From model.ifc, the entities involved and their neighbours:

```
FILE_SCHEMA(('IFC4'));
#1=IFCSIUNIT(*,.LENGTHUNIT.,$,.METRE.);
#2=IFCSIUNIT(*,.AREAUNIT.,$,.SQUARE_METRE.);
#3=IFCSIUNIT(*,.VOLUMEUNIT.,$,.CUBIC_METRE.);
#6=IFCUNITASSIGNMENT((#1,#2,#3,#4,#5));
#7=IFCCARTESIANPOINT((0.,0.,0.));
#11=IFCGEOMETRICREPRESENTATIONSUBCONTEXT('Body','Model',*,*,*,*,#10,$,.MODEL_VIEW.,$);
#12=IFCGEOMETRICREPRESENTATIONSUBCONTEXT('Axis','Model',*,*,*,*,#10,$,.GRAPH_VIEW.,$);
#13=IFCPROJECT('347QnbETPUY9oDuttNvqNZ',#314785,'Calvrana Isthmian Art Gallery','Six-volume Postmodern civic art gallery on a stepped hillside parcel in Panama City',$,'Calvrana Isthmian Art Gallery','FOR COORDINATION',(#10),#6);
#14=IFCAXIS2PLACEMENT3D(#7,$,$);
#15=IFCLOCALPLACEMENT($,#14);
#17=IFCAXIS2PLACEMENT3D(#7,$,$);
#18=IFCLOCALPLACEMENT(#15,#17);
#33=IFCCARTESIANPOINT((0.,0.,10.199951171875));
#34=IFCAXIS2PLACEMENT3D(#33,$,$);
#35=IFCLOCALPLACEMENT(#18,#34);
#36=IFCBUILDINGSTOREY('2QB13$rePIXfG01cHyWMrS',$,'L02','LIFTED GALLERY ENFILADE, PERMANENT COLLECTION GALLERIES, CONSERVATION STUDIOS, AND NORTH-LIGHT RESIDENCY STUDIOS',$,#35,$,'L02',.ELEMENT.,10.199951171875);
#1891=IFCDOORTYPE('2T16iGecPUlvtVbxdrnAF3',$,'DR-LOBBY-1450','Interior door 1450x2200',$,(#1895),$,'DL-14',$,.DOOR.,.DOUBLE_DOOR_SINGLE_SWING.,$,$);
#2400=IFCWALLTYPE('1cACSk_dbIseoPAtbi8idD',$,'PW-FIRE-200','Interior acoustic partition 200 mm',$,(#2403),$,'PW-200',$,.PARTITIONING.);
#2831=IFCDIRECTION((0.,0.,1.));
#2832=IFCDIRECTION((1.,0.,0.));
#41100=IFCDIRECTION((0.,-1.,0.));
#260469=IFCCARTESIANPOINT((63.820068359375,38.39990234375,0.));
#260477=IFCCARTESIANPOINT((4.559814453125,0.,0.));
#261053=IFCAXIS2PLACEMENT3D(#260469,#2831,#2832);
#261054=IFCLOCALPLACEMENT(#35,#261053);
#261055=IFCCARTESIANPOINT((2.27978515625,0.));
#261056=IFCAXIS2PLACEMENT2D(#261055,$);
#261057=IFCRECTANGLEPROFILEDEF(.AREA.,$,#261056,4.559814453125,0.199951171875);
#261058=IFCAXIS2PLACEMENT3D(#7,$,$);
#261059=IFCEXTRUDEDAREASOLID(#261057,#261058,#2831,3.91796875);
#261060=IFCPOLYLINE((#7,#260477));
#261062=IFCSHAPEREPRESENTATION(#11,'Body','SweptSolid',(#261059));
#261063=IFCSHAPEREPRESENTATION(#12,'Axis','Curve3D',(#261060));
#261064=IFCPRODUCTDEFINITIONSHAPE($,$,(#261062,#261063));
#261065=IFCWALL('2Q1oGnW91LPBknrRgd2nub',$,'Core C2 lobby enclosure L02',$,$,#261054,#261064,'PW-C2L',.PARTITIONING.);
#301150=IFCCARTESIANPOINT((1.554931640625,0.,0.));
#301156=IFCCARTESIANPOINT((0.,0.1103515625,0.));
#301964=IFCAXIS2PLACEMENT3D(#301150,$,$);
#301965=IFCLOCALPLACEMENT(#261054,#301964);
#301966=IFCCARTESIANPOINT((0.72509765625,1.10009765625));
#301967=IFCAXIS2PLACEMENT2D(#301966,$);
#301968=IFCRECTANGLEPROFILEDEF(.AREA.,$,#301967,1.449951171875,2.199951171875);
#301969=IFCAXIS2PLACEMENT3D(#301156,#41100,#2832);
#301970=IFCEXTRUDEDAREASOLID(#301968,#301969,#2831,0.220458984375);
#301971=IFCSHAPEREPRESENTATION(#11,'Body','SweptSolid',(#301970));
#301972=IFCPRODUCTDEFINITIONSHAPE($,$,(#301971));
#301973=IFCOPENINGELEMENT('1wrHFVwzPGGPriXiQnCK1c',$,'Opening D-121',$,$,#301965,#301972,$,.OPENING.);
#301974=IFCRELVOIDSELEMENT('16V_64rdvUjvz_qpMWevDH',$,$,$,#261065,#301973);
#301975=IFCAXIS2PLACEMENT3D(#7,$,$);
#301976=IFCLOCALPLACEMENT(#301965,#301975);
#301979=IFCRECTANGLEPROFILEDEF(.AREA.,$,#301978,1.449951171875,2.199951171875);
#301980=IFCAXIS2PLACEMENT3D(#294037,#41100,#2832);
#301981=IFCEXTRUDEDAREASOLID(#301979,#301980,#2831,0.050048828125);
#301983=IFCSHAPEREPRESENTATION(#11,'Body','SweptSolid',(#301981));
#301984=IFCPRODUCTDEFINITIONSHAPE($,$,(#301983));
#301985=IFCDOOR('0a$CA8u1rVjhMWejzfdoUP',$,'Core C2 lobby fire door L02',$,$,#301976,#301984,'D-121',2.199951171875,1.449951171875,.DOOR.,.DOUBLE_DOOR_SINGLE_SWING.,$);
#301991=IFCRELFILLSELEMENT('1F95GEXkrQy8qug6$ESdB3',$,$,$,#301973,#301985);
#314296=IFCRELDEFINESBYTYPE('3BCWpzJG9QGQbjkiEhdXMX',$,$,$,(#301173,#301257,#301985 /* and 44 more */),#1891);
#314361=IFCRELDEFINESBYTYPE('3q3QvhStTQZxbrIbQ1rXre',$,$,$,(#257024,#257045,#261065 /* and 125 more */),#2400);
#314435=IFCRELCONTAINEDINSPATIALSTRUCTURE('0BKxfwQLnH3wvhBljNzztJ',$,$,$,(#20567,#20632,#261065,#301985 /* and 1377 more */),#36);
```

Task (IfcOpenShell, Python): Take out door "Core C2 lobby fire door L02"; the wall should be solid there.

```python
import ifcopenshell
import ifcopenshell.api.feature
import ifcopenshell.api.root
import ifcopenshell.geom
import ifcopenshell.util.shape

model = ifcopenshell.open("model.ifc")
settings = ifcopenshell.geom.settings()


def volume(element):
    """Net volume in cubic metres, openings subtracted."""
    shape = ifcopenshell.geom.create_shape(settings, element)
    return ifcopenshell.util.shape.get_volume(shape.geometry)


door = model.by_id(301985)
opening = door.FillsVoids[0].RelatingOpeningElement
wall = opening.VoidsElements[0].RelatingBuildingElement
before = volume(wall)

ifcopenshell.api.root.remove_product(model, product=door)
ifcopenshell.api.feature.remove_feature(model, feature=opening)

after = volume(wall)

print(f"wall volume {before:.3f} -> {after:.3f} m3")

model.write("model-out.ifc")
```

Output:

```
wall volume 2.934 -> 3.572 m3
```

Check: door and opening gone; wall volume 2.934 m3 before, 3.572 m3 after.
